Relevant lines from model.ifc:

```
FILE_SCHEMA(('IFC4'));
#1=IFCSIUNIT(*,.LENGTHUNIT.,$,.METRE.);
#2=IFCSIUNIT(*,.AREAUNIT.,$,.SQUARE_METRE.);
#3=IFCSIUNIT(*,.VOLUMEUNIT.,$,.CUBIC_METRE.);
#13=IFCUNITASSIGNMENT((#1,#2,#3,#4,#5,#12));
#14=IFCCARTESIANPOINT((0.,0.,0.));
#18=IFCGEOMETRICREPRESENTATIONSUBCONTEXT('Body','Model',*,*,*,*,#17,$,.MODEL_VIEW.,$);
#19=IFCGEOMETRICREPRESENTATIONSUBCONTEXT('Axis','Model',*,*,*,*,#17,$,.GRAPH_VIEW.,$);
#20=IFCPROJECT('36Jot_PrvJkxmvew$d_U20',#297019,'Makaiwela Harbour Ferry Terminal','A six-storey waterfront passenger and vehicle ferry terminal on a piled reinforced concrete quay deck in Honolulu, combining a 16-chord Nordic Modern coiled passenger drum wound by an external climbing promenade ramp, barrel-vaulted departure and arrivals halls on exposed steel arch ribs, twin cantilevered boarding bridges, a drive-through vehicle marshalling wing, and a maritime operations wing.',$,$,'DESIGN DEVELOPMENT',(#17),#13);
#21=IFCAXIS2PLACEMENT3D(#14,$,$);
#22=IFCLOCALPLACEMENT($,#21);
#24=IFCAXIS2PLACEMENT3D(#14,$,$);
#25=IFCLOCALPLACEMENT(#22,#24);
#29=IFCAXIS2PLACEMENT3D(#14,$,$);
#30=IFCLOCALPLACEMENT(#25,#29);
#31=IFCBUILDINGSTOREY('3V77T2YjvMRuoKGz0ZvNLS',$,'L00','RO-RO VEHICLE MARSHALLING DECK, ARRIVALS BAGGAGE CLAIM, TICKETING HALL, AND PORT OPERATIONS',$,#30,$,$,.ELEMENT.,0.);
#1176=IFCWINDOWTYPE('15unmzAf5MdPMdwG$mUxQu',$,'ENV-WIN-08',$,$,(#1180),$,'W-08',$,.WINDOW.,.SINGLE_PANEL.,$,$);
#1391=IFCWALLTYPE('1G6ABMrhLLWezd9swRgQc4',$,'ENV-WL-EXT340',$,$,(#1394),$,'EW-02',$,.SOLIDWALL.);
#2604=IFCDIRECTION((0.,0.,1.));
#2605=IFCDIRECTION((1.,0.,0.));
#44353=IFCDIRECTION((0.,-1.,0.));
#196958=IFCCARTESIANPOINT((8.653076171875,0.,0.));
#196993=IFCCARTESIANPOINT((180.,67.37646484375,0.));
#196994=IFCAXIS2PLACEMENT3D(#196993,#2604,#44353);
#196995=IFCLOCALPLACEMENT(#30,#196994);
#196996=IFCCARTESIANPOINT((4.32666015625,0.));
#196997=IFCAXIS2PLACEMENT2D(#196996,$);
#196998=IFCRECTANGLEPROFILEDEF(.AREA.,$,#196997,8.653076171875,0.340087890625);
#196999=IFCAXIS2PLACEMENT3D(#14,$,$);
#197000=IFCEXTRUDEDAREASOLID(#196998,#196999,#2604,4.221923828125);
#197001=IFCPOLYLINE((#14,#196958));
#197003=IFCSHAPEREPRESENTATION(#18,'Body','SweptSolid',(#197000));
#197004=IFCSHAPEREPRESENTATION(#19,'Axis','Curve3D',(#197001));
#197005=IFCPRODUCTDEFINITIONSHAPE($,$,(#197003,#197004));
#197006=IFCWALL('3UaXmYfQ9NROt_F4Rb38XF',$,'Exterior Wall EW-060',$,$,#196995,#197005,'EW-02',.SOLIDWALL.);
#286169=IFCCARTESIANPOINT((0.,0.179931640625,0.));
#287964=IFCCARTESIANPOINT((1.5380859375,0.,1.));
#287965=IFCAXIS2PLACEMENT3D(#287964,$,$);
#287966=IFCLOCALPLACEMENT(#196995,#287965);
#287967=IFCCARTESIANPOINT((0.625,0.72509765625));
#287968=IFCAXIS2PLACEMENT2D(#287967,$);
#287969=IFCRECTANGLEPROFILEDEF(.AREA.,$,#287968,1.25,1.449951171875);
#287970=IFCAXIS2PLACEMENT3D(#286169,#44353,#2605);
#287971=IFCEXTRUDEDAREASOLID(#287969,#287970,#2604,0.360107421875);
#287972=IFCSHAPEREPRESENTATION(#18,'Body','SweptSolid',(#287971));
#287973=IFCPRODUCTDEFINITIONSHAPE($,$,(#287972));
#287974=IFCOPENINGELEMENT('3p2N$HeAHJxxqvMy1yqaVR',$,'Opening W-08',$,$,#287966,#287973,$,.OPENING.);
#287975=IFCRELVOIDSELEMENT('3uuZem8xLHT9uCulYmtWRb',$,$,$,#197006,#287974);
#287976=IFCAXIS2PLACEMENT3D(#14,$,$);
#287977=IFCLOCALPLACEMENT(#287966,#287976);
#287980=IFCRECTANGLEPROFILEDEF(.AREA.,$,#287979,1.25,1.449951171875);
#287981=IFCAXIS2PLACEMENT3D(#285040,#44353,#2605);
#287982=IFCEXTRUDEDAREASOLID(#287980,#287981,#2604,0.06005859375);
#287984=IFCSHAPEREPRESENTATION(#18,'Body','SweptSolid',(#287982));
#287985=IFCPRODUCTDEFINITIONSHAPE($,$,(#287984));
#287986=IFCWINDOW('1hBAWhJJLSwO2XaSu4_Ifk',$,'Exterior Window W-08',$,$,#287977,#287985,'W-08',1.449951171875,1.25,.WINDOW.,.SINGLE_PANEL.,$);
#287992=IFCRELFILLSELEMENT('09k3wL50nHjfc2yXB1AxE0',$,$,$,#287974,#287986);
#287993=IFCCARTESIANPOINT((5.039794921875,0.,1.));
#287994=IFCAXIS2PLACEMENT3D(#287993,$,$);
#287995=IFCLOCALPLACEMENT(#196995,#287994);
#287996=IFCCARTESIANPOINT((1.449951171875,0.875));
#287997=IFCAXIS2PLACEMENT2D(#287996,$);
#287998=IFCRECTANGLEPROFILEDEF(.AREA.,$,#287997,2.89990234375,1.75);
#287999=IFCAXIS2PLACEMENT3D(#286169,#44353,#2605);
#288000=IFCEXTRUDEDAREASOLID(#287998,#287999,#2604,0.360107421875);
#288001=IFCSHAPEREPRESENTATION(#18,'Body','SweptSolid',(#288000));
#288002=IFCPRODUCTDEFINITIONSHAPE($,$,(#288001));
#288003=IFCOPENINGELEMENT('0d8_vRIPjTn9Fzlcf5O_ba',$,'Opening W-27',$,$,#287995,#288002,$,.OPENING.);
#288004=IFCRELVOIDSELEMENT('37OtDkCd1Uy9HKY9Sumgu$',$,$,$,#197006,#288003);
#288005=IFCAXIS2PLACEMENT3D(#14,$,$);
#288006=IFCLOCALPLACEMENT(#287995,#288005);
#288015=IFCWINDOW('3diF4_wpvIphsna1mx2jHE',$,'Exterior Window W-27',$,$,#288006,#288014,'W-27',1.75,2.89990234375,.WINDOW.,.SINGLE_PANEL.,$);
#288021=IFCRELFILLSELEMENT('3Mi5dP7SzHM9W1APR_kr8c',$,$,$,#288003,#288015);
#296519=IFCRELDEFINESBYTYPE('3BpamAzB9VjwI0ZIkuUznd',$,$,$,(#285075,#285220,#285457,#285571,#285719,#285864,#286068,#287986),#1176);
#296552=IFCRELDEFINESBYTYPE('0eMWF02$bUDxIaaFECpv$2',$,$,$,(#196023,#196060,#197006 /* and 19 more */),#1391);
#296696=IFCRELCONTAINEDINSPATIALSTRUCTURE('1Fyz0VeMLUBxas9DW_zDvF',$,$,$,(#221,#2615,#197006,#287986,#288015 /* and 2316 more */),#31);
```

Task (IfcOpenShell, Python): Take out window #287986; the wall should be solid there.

```python
import ifcopenshell
import ifcopenshell.api.feature
import ifcopenshell.api.root
import ifcopenshell.geom
import ifcopenshell.util.shape

model = ifcopenshell.open("model.ifc")
settings = ifcopenshell.geom.settings()


def volume(element):
    """Net volume in cubic metres, openings subtracted."""
    shape = ifcopenshell.geom.create_shape(settings, element)
    return ifcopenshell.util.shape.get_volume(shape.geometry)


window = model.by_guid("1hBAWhJJLSwO2XaSu4_Ifk")
opening = window.FillsVoids[0].RelatingOpeningElement
wall = opening.VoidsElements[0].RelatingBuildingElement
before = volume(wall)

ifcopenshell.api.root.remove_product(model, product=window)
ifcopenshell.api.feature.remove_feature(model, feature=opening)

after = volume(wall)

print(f"wall volume {before:.3f} -> {after:.3f} m3")

model.write("model-out.ifc")
```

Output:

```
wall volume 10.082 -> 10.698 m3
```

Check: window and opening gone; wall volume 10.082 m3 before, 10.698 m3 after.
